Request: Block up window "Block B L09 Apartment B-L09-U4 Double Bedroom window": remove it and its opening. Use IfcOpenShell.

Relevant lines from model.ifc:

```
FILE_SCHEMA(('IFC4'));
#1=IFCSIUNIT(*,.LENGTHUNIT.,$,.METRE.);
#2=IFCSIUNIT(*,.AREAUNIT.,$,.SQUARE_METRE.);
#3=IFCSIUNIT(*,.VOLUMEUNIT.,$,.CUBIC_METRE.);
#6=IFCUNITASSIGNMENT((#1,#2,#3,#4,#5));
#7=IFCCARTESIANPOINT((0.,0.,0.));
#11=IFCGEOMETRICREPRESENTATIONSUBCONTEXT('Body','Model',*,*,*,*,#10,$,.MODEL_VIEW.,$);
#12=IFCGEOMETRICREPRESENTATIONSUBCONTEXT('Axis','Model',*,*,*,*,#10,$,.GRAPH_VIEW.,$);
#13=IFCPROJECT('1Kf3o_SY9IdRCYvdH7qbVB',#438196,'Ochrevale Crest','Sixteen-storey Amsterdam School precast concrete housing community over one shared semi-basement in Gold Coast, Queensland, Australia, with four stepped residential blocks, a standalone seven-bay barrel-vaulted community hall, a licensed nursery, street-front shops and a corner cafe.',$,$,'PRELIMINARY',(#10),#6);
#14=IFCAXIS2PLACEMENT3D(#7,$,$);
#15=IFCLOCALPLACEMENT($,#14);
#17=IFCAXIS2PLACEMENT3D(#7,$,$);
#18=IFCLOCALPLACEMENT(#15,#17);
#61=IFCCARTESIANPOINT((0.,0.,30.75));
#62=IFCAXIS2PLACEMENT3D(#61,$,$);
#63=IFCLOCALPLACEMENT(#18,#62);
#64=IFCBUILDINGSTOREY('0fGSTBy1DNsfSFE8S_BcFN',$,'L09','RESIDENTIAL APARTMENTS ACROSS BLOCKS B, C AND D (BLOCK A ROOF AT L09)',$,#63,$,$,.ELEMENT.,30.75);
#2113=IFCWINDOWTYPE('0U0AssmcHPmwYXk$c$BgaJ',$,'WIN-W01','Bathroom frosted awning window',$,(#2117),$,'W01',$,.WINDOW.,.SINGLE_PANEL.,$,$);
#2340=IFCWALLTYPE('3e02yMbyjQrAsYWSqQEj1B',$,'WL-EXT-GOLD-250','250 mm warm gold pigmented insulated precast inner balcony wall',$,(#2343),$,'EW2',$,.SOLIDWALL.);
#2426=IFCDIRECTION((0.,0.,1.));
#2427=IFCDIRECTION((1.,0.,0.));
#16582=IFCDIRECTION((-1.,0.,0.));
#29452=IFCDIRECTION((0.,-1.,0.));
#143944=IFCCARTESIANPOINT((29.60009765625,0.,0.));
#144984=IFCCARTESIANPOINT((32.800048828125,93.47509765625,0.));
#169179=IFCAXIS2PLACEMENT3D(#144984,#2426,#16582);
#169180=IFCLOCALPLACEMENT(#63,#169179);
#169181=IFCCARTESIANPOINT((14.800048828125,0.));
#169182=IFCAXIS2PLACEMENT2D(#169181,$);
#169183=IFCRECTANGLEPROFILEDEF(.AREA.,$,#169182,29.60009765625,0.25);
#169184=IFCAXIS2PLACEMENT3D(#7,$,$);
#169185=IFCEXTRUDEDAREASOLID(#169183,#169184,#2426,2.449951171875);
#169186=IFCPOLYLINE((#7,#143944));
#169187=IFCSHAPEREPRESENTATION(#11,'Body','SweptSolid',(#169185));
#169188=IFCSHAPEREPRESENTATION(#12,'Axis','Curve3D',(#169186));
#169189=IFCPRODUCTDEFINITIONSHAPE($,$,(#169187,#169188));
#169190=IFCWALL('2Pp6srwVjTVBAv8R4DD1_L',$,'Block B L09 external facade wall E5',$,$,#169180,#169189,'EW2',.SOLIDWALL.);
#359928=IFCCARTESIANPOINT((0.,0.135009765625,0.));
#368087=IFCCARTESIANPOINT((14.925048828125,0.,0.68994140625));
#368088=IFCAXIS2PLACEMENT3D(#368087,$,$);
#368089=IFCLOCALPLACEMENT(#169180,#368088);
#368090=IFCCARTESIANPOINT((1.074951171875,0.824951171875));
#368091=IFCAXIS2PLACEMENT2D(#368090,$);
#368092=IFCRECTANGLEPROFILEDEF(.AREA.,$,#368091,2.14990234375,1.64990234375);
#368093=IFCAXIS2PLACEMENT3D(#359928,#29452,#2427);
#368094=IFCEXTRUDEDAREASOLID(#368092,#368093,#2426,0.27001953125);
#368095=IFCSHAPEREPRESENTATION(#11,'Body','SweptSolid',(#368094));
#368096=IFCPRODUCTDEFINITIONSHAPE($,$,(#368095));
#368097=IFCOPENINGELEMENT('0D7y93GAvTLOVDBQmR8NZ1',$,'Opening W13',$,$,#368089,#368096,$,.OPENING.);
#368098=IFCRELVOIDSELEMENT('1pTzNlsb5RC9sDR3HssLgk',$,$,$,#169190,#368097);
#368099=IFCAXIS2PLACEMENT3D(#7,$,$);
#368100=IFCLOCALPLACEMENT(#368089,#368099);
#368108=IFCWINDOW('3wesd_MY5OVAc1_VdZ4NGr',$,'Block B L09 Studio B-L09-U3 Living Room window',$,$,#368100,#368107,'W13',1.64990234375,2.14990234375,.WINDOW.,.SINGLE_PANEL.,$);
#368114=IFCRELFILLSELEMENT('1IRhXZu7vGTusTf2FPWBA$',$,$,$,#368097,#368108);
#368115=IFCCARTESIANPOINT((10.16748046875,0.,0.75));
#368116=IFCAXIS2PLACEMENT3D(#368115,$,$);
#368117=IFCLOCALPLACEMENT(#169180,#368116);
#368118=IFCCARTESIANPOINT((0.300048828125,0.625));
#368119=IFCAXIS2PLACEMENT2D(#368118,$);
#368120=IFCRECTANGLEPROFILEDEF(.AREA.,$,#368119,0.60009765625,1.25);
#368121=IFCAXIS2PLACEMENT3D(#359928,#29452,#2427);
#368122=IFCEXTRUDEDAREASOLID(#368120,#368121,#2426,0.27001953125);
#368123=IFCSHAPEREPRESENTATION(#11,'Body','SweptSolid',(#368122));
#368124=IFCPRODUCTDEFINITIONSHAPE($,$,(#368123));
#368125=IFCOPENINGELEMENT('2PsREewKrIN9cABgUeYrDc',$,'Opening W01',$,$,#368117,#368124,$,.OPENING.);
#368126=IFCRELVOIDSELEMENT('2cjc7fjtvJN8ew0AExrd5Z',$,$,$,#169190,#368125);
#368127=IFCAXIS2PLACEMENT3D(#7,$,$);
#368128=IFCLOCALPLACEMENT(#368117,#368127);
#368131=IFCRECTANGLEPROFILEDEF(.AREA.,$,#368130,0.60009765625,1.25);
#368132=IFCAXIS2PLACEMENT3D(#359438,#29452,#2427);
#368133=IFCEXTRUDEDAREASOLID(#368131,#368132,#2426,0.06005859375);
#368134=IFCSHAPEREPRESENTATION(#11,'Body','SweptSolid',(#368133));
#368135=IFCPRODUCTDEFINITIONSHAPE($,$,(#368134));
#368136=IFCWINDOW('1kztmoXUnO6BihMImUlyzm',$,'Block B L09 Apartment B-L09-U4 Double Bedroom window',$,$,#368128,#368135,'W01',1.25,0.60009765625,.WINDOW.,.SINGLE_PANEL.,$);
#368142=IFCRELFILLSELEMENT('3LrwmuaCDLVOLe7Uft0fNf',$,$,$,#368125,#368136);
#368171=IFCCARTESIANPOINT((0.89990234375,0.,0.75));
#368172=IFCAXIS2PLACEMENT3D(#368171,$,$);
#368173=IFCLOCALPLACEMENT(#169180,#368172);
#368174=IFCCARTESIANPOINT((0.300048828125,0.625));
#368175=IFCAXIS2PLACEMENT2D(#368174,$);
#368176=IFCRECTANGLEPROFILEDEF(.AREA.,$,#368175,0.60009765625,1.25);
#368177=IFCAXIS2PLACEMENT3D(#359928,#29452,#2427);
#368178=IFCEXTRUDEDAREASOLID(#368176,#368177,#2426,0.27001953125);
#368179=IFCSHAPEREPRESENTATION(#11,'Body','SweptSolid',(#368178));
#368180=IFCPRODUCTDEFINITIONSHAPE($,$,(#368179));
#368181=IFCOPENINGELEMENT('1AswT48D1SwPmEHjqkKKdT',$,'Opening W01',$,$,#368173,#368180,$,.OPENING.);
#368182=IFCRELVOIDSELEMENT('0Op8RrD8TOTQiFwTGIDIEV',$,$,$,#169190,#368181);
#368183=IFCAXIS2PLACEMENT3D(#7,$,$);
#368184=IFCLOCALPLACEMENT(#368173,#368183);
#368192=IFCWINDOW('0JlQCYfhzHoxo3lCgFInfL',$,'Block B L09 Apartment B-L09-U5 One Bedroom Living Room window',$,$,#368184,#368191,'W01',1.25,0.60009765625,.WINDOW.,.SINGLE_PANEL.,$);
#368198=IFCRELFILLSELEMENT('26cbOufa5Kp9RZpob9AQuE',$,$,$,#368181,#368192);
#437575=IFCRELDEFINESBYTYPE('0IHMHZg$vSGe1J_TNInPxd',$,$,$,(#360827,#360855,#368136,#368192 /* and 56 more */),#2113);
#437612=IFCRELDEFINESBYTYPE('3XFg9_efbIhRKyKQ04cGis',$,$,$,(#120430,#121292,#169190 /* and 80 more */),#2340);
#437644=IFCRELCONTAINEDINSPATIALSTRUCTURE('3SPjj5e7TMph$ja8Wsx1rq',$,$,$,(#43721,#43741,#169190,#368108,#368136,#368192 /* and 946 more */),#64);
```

```python
import ifcopenshell
import ifcopenshell.api.feature
import ifcopenshell.api.root
import ifcopenshell.geom
import ifcopenshell.util.shape

model = ifcopenshell.open("model.ifc")
settings = ifcopenshell.geom.settings()


def volume(element):
    """Net volume in cubic metres, openings subtracted."""
    shape = ifcopenshell.geom.create_shape(settings, element)
    return ifcopenshell.util.shape.get_volume(shape.geometry)


window = model.by_id(368136)
opening = window.FillsVoids[0].RelatingOpeningElement
wall = opening.VoidsElements[0].RelatingBuildingElement
before = volume(wall)

ifcopenshell.api.root.remove_product(model, product=window)
ifcopenshell.api.feature.remove_feature(model, feature=opening)

after = volume(wall)

print(f"wall volume {before:.3f} -> {after:.3f} m3")

model.write("model_v2.ifc")
```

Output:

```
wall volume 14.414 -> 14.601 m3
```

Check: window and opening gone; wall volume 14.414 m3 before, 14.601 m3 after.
